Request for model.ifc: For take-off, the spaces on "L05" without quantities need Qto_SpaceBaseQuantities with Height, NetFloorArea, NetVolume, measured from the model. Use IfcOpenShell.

First a look at what the model holds.

```python
import ifcopenshell
import ifcopenshell.util.element
import ifcopenshell.util.unit

model = ifcopenshell.open("model.ifc")
print(model.schema)
for unit_type in ("LENGTHUNIT", "AREAUNIT", "VOLUMEUNIT"):
    print(unit_type, ifcopenshell.util.unit.calculate_unit_scale(model, unit_type))
storey = next(s for s in model.by_type("IfcBuildingStorey") if s.Name == "L05")
spaces = [e for e in ifcopenshell.util.element.get_decomposition(storey) if e.is_a("IfcSpace")]
for e in sorted(spaces, key=lambda e: e.id()):
    print(e.id(), e.is_a(), e.Name, list(ifcopenshell.util.element.get_psets(e, qtos_only=True)), sep=" | ")
```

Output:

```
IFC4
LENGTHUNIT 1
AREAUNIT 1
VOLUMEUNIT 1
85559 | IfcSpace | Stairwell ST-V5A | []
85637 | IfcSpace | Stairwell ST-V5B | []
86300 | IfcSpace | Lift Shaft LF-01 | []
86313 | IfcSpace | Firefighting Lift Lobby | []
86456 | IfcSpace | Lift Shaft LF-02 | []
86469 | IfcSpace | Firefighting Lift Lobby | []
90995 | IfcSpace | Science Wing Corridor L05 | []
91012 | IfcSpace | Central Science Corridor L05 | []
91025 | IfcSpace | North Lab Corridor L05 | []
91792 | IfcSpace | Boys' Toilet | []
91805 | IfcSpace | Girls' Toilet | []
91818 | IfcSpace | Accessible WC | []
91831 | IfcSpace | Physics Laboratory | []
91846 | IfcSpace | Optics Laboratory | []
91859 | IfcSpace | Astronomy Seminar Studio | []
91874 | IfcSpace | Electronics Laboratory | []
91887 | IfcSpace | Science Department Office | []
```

```python
import ifcopenshell
import ifcopenshell.api.pset
import ifcopenshell.geom
import ifcopenshell.util.element
import ifcopenshell.util.shape
import ifcopenshell.util.unit

model = ifcopenshell.open("model.ifc")
unit_scale = ifcopenshell.util.unit.calculate_unit_scale(model)
area_scale = ifcopenshell.util.unit.calculate_unit_scale(model, "AREAUNIT")
volume_scale = ifcopenshell.util.unit.calculate_unit_scale(model, "VOLUMEUNIT")
settings = ifcopenshell.geom.settings()

storey = next(s for s in model.by_type("IfcBuildingStorey") if s.Name == "L05")
spaces = [e for e in ifcopenshell.util.element.get_decomposition(storey) if e.is_a("IfcSpace")]

for e in sorted(spaces, key=lambda e: e.id()):
    if ifcopenshell.util.element.get_psets(e, qtos_only=True, should_inherit=False):
        continue
    # Geometry comes back in metres, in the element's own axes.
    shape = ifcopenshell.geom.create_shape(settings, e)
    values = {
        "Height": ifcopenshell.util.shape.get_z(shape.geometry) / unit_scale,
        "NetFloorArea": ifcopenshell.util.shape.get_footprint_area(shape.geometry) / area_scale,
        "NetVolume": ifcopenshell.util.shape.get_volume(shape.geometry) / volume_scale,
    }
    qto = ifcopenshell.api.pset.add_qto(model, product=e, name="Qto_SpaceBaseQuantities")
    ifcopenshell.api.pset.edit_qto(model, qto=qto, properties=values)
    print(e.id(), {k: round(v, 3) for k, v in values.items()})

model.write("model_rev.ifc")
```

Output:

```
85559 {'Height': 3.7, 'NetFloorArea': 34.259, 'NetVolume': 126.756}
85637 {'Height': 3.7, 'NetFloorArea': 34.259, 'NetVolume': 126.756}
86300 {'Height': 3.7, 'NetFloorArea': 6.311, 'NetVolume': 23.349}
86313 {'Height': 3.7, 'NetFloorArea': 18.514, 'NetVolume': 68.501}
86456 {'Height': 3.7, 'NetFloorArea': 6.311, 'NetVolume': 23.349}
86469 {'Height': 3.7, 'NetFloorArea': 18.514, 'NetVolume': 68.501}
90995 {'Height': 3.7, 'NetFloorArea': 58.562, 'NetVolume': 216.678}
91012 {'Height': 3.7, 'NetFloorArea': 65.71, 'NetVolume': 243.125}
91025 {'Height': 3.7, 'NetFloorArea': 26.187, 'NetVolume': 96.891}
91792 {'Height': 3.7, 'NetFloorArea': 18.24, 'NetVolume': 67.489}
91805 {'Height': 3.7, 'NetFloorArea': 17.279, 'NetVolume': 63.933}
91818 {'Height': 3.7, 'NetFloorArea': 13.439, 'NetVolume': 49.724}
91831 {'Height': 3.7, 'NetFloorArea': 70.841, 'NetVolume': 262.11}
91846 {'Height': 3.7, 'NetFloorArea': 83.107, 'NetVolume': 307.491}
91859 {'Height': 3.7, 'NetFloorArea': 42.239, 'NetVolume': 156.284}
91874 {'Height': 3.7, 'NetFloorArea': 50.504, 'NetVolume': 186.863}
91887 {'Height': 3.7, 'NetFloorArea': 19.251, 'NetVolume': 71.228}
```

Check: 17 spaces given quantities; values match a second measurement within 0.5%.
